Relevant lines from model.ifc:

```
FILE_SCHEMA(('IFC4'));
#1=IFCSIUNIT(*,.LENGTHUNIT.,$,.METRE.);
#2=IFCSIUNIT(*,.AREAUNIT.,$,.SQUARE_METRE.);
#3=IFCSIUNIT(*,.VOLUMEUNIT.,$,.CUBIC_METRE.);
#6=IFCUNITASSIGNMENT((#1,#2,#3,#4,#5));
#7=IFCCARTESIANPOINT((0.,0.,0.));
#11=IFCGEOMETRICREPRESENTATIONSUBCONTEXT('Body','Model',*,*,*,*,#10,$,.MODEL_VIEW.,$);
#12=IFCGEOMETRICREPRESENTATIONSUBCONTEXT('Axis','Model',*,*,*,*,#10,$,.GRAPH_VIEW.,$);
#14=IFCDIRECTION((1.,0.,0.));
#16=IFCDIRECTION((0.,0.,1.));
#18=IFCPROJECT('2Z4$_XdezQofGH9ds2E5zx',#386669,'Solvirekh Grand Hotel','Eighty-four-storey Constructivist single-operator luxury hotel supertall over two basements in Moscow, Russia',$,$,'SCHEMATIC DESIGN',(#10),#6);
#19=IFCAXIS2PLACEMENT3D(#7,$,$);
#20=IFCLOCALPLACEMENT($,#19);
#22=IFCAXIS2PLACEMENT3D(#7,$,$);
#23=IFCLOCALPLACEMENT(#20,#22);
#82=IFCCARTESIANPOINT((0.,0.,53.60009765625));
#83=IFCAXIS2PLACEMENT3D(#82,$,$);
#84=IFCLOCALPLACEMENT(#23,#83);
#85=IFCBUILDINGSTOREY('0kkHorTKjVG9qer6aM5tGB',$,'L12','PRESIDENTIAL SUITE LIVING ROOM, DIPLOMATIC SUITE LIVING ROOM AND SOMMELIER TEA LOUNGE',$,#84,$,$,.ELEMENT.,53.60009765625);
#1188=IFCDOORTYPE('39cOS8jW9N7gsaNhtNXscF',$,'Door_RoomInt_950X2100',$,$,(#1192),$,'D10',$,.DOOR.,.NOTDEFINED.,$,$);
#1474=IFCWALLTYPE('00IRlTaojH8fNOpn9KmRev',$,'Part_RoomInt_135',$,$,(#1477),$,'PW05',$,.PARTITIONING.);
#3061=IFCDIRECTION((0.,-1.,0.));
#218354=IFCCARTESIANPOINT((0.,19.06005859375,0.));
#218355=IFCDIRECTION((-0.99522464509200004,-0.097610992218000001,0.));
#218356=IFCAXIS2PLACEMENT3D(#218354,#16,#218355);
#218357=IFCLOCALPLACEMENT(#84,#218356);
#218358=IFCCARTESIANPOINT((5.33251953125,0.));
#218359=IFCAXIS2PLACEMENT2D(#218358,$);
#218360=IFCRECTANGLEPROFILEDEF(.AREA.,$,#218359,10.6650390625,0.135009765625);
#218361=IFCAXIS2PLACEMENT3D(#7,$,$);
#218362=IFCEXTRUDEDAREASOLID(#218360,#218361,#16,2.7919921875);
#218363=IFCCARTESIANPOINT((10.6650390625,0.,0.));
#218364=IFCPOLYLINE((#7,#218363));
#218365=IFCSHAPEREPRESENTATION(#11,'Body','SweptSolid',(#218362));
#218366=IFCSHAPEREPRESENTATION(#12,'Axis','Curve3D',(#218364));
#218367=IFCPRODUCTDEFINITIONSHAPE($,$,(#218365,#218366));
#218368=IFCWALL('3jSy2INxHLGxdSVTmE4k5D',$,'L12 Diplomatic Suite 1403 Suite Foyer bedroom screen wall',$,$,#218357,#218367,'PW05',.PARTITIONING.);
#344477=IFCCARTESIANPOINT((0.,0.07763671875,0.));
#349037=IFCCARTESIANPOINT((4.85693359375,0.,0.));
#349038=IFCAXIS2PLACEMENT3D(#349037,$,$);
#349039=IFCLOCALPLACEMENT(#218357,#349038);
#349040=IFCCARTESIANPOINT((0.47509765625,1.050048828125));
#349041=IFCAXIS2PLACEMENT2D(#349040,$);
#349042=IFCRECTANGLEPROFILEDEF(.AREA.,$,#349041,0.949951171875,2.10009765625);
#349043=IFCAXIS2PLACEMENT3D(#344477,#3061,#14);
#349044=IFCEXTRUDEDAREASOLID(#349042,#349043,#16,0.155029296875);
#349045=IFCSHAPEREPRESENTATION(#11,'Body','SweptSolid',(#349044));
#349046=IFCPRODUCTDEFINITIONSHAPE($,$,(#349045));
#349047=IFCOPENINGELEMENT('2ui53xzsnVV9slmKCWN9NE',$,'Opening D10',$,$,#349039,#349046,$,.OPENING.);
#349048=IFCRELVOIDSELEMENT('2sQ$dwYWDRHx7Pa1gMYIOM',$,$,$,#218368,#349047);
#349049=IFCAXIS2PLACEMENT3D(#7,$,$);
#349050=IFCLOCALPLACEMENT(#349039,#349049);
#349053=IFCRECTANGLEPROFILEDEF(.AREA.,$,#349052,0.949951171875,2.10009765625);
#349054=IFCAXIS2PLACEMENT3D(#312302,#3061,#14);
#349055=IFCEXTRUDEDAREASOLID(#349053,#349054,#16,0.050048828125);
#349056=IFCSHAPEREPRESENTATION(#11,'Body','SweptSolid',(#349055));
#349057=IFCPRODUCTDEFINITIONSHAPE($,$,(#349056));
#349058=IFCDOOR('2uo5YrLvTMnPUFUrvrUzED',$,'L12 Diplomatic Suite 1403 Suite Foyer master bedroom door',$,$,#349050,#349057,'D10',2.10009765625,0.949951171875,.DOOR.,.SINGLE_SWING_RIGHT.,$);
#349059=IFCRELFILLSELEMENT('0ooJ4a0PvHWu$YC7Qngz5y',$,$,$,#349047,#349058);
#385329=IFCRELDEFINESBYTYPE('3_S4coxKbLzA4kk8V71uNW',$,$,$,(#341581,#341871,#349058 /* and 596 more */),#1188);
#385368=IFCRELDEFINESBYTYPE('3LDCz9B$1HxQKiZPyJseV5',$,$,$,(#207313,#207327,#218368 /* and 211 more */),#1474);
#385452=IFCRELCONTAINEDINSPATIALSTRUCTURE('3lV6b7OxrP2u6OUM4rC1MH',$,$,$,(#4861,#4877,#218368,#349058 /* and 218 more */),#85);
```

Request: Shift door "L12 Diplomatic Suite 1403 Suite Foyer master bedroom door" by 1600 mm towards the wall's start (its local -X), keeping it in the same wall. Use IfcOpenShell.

```python
import ifcopenshell
import ifcopenshell.api.geometry
import ifcopenshell.util.placement
import ifcopenshell.util.unit

model = ifcopenshell.open("model.ifc")
unit_scale = ifcopenshell.util.unit.calculate_unit_scale(model)

door = model.by_guid("2uo5YrLvTMnPUFUrvrUzED")
opening = door.FillsVoids[0].RelatingOpeningElement
wall = opening.VoidsElements[0].RelatingBuildingElement

wall_matrix = ifcopenshell.util.placement.get_local_placement(wall.ObjectPlacement)
shift = wall_matrix[:3, 0] * -1.6 / unit_scale
before = ifcopenshell.util.placement.get_local_placement(door.ObjectPlacement)[:3, 3].copy()

# The door is placed relative to its opening, so it follows when the opening moves.
matrix = ifcopenshell.util.placement.get_local_placement(opening.ObjectPlacement)
matrix[:3, 3] += shift
ifcopenshell.api.geometry.edit_object_placement(
    model, product=opening, matrix=matrix, is_si=False, should_transform_children=True
)

after = ifcopenshell.util.placement.get_local_placement(door.ObjectPlacement)[:3, 3]
print("door moved by", (after - before).round(3) + 0.0)

model.write("model_v2.ifc")
```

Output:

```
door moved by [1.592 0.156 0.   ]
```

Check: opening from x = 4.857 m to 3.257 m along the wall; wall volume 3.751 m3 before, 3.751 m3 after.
